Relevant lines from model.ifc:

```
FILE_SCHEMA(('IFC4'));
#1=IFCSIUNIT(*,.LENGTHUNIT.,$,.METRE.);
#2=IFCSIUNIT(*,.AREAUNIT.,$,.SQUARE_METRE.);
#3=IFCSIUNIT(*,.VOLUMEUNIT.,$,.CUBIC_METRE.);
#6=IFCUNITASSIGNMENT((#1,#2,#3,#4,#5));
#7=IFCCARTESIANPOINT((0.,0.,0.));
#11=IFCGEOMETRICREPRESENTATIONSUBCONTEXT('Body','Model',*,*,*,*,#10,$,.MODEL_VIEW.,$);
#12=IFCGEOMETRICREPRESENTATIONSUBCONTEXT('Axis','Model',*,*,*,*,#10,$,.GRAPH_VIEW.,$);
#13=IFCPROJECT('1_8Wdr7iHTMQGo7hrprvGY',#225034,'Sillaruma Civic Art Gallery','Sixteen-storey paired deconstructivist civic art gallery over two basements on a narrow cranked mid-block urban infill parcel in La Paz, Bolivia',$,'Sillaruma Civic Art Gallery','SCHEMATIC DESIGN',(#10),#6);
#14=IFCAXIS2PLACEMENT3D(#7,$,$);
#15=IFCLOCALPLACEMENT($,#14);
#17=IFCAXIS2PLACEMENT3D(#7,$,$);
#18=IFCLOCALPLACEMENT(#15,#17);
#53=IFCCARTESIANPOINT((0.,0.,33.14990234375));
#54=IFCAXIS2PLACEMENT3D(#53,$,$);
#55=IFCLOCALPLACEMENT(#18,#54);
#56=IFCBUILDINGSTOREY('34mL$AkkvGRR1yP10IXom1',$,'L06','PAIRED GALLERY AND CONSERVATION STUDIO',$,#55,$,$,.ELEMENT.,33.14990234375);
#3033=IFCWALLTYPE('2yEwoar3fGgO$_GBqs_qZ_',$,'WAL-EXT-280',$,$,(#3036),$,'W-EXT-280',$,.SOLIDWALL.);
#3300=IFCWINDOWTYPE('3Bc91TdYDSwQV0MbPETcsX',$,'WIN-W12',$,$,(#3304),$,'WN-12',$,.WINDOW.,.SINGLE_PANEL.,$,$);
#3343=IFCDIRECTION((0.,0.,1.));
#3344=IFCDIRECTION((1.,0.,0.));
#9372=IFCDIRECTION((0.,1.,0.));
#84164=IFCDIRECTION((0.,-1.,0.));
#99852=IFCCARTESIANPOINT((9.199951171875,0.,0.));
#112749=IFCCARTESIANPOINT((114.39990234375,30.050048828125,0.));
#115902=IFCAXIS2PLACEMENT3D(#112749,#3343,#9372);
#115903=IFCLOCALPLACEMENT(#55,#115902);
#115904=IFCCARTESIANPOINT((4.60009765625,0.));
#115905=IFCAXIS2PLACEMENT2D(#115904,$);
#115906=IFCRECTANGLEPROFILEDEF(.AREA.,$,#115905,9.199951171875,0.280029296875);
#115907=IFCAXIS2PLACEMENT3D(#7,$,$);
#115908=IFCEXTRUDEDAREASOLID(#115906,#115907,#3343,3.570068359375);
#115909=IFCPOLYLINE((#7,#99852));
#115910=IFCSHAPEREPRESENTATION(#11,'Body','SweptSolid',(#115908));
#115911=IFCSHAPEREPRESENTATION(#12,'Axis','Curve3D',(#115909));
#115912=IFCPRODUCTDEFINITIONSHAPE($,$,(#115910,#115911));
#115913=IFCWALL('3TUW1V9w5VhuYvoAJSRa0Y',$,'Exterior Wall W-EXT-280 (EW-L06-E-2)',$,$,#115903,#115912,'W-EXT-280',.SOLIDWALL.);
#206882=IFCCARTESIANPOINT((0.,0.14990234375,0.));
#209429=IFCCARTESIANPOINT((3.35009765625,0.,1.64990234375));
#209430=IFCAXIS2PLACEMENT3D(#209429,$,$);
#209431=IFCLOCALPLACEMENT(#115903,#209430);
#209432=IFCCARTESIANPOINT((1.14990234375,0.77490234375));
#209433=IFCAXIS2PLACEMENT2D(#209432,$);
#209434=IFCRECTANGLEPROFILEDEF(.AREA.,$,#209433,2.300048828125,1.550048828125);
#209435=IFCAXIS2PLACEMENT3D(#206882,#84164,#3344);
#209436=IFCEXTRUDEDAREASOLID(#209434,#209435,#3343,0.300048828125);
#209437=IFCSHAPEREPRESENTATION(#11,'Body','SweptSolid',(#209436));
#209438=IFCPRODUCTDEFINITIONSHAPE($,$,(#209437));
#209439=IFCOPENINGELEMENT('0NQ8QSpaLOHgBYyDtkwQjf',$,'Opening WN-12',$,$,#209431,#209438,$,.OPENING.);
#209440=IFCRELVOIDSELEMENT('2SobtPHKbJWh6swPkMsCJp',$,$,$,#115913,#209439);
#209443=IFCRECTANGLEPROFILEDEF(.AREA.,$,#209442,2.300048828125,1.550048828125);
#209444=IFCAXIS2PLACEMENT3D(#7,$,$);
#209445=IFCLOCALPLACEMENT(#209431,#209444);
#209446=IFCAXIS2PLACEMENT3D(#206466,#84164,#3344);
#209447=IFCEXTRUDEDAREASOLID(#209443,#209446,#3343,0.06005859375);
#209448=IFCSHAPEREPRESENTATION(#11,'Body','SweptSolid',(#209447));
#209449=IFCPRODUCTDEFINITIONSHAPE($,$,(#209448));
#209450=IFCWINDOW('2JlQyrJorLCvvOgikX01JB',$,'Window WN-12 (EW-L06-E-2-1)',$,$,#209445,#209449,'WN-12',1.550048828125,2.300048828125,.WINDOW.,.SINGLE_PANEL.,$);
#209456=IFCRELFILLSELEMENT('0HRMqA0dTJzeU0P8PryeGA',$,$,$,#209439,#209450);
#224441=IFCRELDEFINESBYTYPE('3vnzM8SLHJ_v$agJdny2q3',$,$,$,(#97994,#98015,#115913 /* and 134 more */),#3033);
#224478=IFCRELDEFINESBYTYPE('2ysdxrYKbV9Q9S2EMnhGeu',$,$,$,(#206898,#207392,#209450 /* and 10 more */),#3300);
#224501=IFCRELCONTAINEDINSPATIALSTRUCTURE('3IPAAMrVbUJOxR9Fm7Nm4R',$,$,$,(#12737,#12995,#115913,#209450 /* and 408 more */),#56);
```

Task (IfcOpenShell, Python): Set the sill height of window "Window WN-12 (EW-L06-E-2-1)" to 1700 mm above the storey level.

```python
import numpy as np
import ifcopenshell
import ifcopenshell.api.geometry
import ifcopenshell.geom
import ifcopenshell.util.element
import ifcopenshell.util.placement
import ifcopenshell.util.shape
import ifcopenshell.util.unit

model = ifcopenshell.open("model.ifc")
unit_scale = ifcopenshell.util.unit.calculate_unit_scale(model)

window = model.by_guid("2JlQyrJorLCvvOgikX01JB")
opening = window.FillsVoids[0].RelatingOpeningElement
storey = ifcopenshell.util.element.get_container(window, ifc_class="IfcBuildingStorey")
level = ifcopenshell.util.placement.get_local_placement(storey.ObjectPlacement)[2, 3]

# The opening's origin need not be at the sill, so measure its lowest point.
shape = ifcopenshell.geom.create_shape(ifcopenshell.geom.settings(), opening)
bottom = ifcopenshell.util.shape.get_shape_bottom_elevation(shape, shape.geometry) / unit_scale
dz = level + 1.7 - bottom

shift = np.array([0.0, 0.0, dz])
# The window is placed relative to its opening, so it follows when the opening moves.
matrix = ifcopenshell.util.placement.get_local_placement(opening.ObjectPlacement)
matrix[:3, 3] += shift
ifcopenshell.api.geometry.edit_object_placement(
    model, product=opening, matrix=matrix, is_si=False, should_transform_children=True
)

print(f"moved by {dz * unit_scale:+.3f} m")

model.write("model_edited.ifc")
```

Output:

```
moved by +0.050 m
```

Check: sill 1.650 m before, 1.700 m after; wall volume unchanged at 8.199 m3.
